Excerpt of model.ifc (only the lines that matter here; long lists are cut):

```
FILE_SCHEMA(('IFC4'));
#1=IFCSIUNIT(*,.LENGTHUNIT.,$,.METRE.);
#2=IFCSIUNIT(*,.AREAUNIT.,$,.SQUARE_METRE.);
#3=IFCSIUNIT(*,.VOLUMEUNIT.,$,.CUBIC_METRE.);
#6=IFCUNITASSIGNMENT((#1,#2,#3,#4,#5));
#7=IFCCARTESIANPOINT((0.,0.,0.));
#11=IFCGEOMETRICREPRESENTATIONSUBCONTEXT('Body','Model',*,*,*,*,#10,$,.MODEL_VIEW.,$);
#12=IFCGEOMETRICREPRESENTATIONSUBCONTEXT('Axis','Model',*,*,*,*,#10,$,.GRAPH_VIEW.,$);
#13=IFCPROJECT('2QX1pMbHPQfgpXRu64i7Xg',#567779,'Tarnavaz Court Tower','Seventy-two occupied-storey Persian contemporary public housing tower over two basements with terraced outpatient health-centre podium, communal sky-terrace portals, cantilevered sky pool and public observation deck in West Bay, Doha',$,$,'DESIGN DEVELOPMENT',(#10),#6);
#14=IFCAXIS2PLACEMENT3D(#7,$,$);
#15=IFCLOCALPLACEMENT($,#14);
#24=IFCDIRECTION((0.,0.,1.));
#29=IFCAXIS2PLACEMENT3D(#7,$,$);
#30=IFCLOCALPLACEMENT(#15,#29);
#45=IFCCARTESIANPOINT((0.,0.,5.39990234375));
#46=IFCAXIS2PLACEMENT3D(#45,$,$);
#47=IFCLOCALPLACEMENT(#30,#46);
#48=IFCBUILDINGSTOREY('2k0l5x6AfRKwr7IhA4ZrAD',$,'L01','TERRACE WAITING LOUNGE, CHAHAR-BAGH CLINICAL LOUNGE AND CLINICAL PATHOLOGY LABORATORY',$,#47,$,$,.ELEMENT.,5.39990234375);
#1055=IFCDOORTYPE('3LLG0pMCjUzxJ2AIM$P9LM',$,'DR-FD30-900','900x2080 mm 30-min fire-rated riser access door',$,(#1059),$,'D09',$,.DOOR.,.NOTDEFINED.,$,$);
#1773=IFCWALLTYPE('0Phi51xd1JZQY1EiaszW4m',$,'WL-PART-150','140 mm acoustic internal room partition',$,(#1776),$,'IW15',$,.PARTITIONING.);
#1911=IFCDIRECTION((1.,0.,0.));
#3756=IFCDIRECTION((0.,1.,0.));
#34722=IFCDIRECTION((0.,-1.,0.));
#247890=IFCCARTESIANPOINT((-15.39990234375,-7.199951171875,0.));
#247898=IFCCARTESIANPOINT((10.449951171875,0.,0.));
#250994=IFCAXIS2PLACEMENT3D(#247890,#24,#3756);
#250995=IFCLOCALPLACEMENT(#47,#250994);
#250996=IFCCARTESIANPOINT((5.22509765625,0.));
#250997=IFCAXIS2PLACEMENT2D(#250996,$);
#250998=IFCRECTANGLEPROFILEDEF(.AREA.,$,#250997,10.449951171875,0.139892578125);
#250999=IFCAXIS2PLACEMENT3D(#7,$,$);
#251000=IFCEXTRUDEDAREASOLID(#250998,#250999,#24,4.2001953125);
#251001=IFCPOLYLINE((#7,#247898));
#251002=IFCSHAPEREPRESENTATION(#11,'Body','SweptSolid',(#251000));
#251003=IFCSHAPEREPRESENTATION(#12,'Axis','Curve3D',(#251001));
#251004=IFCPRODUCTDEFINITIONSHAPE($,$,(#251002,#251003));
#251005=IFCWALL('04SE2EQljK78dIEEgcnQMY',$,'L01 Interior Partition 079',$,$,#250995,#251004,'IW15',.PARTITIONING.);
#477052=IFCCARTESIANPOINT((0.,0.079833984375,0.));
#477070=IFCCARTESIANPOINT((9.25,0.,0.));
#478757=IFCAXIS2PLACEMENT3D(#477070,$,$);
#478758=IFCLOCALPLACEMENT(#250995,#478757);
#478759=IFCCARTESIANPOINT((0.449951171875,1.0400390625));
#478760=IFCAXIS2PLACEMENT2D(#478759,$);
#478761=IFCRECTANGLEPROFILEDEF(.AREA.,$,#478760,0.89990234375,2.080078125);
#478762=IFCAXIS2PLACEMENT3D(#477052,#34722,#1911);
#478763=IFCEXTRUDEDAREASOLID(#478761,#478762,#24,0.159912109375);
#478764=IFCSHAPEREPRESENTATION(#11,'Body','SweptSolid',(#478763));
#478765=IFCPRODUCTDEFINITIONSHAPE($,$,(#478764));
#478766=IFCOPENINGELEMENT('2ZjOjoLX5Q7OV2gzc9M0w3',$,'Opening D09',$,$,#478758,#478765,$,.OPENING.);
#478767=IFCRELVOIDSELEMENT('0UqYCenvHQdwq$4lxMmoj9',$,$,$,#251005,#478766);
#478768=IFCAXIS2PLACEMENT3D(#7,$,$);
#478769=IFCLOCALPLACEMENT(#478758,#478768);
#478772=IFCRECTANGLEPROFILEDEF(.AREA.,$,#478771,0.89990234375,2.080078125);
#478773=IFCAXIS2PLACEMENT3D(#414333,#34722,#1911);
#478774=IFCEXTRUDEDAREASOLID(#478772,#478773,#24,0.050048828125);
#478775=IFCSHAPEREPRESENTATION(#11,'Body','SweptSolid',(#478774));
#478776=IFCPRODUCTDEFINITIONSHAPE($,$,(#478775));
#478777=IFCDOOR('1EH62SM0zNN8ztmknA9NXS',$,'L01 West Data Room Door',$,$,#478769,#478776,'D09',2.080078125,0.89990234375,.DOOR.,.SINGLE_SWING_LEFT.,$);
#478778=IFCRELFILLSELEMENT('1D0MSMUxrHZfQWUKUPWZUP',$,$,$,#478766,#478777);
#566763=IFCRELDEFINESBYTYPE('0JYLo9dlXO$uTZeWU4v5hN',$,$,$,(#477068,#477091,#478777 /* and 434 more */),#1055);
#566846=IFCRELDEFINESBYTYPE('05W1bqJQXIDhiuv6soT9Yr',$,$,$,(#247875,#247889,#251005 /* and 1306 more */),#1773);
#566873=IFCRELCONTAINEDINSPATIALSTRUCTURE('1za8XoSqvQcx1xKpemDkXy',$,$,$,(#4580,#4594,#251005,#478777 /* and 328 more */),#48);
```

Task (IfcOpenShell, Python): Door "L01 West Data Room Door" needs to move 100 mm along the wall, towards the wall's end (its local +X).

```python
import ifcopenshell
import ifcopenshell.api.geometry
import ifcopenshell.util.placement

model = ifcopenshell.open("model.ifc")

door = model.by_guid("1EH62SM0zNN8ztmknA9NXS")
opening = door.FillsVoids[0].RelatingOpeningElement
wall = opening.VoidsElements[0].RelatingBuildingElement

wall_matrix = ifcopenshell.util.placement.get_local_placement(wall.ObjectPlacement)
shift = wall_matrix[:3, 0] * 0.1
before = ifcopenshell.util.placement.get_local_placement(door.ObjectPlacement)[:3, 3].copy()

# The door is placed relative to its opening, so it follows when the opening moves.
matrix = ifcopenshell.util.placement.get_local_placement(opening.ObjectPlacement)
matrix[:3, 3] += shift
ifcopenshell.api.geometry.edit_object_placement(
    model, product=opening, matrix=matrix, is_si=False, should_transform_children=True
)

after = ifcopenshell.util.placement.get_local_placement(door.ObjectPlacement)[:3, 3]
print("door moved by", (after - before).round(3) + 0.0)

model.write("model_updated.ifc")
```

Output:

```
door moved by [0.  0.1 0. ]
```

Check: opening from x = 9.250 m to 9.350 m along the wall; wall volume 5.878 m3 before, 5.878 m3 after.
